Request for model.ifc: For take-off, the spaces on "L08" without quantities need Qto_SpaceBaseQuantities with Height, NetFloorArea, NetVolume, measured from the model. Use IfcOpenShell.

First a look at what the model holds.

```python
import ifcopenshell
import ifcopenshell.util.element
import ifcopenshell.util.unit

model = ifcopenshell.open("model.ifc")
print(model.schema)
for unit_type in ("LENGTHUNIT", "AREAUNIT", "VOLUMEUNIT"):
    print(unit_type, ifcopenshell.util.unit.calculate_unit_scale(model, unit_type))
storey = next(s for s in model.by_type("IfcBuildingStorey") if s.Name == "L08")
spaces = [e for e in ifcopenshell.util.element.get_decomposition(storey) if e.is_a("IfcSpace")]
for e in sorted(spaces, key=lambda e: e.id()):
    print(e.id(), e.is_a(), e.Name, list(ifcopenshell.util.element.get_psets(e, qtos_only=True)), sep=" | ")
```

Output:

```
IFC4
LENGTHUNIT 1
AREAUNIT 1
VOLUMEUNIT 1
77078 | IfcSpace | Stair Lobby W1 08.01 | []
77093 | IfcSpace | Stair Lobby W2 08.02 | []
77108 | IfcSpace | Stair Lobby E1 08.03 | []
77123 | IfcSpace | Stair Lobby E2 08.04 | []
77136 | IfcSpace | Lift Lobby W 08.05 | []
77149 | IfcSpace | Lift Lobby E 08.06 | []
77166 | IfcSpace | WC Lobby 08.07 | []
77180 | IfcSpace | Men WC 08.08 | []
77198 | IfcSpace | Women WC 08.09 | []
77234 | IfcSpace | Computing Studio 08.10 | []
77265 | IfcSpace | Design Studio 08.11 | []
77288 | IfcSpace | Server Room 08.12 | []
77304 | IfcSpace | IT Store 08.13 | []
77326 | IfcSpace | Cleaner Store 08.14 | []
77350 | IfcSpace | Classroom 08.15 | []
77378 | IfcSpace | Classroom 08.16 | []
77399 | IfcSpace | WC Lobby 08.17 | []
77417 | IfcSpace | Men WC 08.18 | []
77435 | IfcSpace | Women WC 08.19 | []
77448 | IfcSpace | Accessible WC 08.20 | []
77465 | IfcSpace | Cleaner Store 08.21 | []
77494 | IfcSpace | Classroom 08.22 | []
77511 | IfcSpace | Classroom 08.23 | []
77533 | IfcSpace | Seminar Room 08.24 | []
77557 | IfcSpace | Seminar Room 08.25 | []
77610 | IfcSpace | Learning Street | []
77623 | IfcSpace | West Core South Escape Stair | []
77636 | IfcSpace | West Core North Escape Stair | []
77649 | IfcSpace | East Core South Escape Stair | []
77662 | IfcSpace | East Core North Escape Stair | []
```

```python
import ifcopenshell
import ifcopenshell.api.pset
import ifcopenshell.geom
import ifcopenshell.util.element
import ifcopenshell.util.shape
import ifcopenshell.util.unit

model = ifcopenshell.open("model.ifc")
unit_scale = ifcopenshell.util.unit.calculate_unit_scale(model)
area_scale = ifcopenshell.util.unit.calculate_unit_scale(model, "AREAUNIT")
volume_scale = ifcopenshell.util.unit.calculate_unit_scale(model, "VOLUMEUNIT")
settings = ifcopenshell.geom.settings()

storey = next(s for s in model.by_type("IfcBuildingStorey") if s.Name == "L08")
spaces = [e for e in ifcopenshell.util.element.get_decomposition(storey) if e.is_a("IfcSpace")]

for e in sorted(spaces, key=lambda e: e.id()):
    if ifcopenshell.util.element.get_psets(e, qtos_only=True, should_inherit=False):
        continue
    # Geometry comes back in metres, in the element's own axes.
    shape = ifcopenshell.geom.create_shape(settings, e)
    values = {
        "Height": ifcopenshell.util.shape.get_z(shape.geometry) / unit_scale,
        "NetFloorArea": ifcopenshell.util.shape.get_footprint_area(shape.geometry) / area_scale,
        "NetVolume": ifcopenshell.util.shape.get_volume(shape.geometry) / volume_scale,
    }
    qto = ifcopenshell.api.pset.add_qto(model, product=e, name="Qto_SpaceBaseQuantities")
    ifcopenshell.api.pset.edit_qto(model, qto=qto, properties=values)
    print(e.id(), {k: round(v, 3) for k, v in values.items()})

model.write("model_updated.ifc")
```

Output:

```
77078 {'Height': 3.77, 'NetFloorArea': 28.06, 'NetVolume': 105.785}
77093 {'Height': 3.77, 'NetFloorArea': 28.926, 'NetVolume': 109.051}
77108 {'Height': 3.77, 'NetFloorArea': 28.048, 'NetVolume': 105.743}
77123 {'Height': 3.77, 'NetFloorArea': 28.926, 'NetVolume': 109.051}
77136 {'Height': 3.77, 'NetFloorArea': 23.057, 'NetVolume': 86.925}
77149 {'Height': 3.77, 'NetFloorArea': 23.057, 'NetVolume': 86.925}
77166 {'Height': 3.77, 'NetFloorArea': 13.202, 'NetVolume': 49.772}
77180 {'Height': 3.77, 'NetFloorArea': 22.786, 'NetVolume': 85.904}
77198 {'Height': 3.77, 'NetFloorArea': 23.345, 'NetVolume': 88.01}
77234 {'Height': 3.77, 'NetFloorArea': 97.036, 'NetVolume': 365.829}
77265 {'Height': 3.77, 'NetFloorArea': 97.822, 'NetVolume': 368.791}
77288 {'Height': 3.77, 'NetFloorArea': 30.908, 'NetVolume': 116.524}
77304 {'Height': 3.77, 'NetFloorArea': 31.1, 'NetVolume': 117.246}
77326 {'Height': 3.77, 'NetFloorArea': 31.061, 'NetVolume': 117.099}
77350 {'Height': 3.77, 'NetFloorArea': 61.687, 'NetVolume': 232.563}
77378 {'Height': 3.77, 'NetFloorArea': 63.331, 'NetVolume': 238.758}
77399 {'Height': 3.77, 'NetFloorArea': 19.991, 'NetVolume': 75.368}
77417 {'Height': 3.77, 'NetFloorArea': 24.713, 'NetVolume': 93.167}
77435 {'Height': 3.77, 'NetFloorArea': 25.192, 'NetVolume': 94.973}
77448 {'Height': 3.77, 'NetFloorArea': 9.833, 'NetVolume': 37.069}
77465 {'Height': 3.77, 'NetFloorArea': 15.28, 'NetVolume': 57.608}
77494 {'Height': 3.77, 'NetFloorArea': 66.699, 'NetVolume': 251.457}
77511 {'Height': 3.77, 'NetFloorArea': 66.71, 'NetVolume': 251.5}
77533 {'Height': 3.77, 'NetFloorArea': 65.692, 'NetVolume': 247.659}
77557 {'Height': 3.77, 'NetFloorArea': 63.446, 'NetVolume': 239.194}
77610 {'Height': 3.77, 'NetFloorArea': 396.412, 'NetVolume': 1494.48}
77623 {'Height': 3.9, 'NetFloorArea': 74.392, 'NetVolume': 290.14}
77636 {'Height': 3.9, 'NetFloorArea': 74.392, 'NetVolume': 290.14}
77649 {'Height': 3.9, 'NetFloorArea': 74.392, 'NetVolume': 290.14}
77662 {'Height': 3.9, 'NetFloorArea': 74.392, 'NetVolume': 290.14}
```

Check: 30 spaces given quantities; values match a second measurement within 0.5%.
